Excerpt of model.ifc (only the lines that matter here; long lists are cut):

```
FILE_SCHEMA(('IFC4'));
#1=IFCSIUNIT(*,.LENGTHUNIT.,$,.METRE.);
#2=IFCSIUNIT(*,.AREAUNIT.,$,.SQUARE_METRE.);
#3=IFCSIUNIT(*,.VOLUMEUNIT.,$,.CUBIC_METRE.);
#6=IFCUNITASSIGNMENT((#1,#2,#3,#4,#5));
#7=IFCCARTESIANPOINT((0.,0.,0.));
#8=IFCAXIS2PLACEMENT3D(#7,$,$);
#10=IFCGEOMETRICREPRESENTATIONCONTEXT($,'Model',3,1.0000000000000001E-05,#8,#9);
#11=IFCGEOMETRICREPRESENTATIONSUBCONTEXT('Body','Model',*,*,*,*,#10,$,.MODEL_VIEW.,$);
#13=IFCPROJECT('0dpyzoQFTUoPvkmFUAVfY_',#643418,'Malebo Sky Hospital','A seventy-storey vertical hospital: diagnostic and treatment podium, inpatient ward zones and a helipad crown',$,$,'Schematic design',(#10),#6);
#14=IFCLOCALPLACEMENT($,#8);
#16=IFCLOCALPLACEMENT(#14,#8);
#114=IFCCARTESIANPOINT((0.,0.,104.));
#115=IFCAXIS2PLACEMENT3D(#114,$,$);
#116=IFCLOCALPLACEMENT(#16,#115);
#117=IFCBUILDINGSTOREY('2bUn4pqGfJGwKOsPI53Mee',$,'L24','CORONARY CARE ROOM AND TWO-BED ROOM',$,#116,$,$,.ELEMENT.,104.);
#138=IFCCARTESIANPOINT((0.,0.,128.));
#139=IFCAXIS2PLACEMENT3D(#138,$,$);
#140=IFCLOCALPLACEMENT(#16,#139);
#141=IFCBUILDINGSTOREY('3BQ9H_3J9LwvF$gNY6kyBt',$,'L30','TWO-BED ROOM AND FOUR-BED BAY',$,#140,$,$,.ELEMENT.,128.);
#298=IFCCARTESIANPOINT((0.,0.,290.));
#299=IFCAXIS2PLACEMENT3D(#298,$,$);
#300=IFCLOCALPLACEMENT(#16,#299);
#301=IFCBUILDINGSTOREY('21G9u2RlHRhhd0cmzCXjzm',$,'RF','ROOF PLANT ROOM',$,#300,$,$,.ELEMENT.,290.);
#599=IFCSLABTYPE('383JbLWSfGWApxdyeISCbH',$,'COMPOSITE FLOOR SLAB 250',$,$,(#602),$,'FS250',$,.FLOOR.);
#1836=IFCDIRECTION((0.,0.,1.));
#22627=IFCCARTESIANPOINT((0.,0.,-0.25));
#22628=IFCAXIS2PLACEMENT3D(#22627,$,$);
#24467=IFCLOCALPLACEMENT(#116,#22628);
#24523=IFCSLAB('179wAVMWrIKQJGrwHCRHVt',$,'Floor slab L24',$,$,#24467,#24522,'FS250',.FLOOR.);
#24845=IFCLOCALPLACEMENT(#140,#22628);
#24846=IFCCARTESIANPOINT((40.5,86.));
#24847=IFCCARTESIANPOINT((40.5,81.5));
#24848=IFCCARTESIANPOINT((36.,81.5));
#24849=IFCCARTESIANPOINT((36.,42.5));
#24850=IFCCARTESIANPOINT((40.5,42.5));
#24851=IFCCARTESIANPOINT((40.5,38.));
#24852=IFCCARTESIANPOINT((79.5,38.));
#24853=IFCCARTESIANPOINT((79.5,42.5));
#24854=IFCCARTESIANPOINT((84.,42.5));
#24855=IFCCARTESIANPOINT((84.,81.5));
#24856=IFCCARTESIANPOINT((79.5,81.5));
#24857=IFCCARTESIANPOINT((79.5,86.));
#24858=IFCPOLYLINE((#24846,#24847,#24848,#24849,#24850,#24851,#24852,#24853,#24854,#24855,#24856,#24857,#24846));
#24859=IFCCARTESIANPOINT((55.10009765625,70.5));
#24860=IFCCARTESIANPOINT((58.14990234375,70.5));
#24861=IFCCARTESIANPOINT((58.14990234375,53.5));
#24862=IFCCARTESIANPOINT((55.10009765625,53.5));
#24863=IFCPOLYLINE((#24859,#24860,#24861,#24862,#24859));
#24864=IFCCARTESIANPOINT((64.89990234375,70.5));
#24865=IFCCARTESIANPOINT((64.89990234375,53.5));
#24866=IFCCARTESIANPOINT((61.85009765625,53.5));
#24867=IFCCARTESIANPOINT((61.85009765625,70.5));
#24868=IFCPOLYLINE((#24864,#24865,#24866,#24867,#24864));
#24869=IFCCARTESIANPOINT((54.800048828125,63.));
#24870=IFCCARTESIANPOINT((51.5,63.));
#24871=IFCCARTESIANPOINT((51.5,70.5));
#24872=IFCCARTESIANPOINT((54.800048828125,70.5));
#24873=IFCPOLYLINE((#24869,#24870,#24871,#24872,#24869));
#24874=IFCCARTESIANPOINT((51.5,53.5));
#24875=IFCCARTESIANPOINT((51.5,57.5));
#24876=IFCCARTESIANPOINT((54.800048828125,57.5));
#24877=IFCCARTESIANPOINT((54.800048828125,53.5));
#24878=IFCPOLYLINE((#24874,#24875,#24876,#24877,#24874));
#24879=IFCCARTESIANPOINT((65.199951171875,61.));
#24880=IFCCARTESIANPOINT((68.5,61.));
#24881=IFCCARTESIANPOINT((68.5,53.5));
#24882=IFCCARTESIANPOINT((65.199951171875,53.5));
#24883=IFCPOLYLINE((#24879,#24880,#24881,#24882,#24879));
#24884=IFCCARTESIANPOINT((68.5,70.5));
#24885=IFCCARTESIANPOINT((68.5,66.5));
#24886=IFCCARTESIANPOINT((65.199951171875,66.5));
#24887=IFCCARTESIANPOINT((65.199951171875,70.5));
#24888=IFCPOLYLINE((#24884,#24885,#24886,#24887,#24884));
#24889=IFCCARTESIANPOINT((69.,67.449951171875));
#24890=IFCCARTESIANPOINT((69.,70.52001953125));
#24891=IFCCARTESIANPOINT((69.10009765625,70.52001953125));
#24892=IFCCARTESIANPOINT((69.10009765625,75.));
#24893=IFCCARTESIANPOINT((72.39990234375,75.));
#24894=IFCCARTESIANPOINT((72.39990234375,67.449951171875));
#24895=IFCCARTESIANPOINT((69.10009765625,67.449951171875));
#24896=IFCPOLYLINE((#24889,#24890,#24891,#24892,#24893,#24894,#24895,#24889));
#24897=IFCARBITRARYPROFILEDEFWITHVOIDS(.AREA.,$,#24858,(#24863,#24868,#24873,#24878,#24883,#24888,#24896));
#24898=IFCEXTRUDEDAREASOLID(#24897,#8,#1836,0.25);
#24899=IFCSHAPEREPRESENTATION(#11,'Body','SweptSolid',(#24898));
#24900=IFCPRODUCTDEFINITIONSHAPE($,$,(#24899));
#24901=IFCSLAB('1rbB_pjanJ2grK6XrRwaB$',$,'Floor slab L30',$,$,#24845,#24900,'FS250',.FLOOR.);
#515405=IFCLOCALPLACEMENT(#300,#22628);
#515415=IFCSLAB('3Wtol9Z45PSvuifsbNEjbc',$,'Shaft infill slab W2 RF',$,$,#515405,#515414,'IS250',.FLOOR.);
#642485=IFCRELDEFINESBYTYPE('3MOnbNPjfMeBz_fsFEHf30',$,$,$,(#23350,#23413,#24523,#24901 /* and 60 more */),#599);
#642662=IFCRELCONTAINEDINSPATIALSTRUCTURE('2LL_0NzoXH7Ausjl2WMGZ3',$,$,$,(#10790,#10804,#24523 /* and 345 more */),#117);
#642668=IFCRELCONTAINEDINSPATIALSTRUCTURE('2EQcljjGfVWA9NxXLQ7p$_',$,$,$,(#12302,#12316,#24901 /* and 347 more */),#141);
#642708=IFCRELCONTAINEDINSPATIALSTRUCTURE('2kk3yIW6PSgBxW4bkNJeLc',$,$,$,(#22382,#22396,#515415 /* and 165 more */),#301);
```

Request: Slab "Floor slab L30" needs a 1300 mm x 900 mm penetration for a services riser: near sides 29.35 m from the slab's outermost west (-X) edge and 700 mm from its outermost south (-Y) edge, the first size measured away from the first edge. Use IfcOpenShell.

```python
import numpy as np
import ifcopenshell
import ifcopenshell.api.feature
import ifcopenshell.api.geometry
import ifcopenshell.api.root
import ifcopenshell.geom
import ifcopenshell.util.placement
import ifcopenshell.util.representation
import ifcopenshell.util.shape
import ifcopenshell.util.unit

model = ifcopenshell.open("model.ifc")
unit_scale = ifcopenshell.util.unit.calculate_unit_scale(model)
settings = ifcopenshell.geom.settings()


def volume(element):
    """Net volume in cubic metres, openings subtracted."""
    shape = ifcopenshell.geom.create_shape(settings, element)
    return ifcopenshell.util.shape.get_volume(shape.geometry)


slab = model.by_guid("1rbB_pjanJ2grK6XrRwaB$")
before = volume(slab)

# Extent in the slab's own axes, in metres. The edges named are its -X and -Y sides.
slab_shape = ifcopenshell.geom.create_shape(settings, slab)
vertices = ifcopenshell.util.shape.get_vertices(slab_shape.geometry)
x_min, y_min, bottom = vertices.min(axis=0)
top = vertices[:, 2].max()

opening = ifcopenshell.api.root.create_entity(model, ifc_class="IfcOpeningElement", name="Services riser opening", predefined_type="OPENING")
context = ifcopenshell.util.representation.get_context(model, "Model", "Body", "MODEL_VIEW")
width, depth = 1.3, 0.9
outline = [(0.0, 0.0), (width, 0.0), (width, depth), (0.0, depth), (0.0, 0.0)]
# Overshoot both faces by 50 mm so the cut is clean.
shape = ifcopenshell.api.geometry.add_slab_representation(
    model, context=context, depth=top - bottom + 0.1, polyline=outline
)
ifcopenshell.api.geometry.assign_representation(model, product=opening, representation=shape)

matrix = ifcopenshell.util.placement.get_local_placement(slab.ObjectPlacement)
matrix[:, 3] = matrix @ np.append(np.array([x_min + 29.35, y_min + 0.7, bottom - 0.05]) / unit_scale, 1.0)
ifcopenshell.api.geometry.edit_object_placement(model, product=opening, matrix=matrix, is_si=False)
ifcopenshell.api.feature.add_feature(model, feature=opening, element=slab)

after = volume(slab)

print(f"slab volume {before:.3f} -> {after:.3f} m3")

model.write("model-out.ifc")
```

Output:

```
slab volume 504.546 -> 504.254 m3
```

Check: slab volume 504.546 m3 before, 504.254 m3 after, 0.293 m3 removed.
